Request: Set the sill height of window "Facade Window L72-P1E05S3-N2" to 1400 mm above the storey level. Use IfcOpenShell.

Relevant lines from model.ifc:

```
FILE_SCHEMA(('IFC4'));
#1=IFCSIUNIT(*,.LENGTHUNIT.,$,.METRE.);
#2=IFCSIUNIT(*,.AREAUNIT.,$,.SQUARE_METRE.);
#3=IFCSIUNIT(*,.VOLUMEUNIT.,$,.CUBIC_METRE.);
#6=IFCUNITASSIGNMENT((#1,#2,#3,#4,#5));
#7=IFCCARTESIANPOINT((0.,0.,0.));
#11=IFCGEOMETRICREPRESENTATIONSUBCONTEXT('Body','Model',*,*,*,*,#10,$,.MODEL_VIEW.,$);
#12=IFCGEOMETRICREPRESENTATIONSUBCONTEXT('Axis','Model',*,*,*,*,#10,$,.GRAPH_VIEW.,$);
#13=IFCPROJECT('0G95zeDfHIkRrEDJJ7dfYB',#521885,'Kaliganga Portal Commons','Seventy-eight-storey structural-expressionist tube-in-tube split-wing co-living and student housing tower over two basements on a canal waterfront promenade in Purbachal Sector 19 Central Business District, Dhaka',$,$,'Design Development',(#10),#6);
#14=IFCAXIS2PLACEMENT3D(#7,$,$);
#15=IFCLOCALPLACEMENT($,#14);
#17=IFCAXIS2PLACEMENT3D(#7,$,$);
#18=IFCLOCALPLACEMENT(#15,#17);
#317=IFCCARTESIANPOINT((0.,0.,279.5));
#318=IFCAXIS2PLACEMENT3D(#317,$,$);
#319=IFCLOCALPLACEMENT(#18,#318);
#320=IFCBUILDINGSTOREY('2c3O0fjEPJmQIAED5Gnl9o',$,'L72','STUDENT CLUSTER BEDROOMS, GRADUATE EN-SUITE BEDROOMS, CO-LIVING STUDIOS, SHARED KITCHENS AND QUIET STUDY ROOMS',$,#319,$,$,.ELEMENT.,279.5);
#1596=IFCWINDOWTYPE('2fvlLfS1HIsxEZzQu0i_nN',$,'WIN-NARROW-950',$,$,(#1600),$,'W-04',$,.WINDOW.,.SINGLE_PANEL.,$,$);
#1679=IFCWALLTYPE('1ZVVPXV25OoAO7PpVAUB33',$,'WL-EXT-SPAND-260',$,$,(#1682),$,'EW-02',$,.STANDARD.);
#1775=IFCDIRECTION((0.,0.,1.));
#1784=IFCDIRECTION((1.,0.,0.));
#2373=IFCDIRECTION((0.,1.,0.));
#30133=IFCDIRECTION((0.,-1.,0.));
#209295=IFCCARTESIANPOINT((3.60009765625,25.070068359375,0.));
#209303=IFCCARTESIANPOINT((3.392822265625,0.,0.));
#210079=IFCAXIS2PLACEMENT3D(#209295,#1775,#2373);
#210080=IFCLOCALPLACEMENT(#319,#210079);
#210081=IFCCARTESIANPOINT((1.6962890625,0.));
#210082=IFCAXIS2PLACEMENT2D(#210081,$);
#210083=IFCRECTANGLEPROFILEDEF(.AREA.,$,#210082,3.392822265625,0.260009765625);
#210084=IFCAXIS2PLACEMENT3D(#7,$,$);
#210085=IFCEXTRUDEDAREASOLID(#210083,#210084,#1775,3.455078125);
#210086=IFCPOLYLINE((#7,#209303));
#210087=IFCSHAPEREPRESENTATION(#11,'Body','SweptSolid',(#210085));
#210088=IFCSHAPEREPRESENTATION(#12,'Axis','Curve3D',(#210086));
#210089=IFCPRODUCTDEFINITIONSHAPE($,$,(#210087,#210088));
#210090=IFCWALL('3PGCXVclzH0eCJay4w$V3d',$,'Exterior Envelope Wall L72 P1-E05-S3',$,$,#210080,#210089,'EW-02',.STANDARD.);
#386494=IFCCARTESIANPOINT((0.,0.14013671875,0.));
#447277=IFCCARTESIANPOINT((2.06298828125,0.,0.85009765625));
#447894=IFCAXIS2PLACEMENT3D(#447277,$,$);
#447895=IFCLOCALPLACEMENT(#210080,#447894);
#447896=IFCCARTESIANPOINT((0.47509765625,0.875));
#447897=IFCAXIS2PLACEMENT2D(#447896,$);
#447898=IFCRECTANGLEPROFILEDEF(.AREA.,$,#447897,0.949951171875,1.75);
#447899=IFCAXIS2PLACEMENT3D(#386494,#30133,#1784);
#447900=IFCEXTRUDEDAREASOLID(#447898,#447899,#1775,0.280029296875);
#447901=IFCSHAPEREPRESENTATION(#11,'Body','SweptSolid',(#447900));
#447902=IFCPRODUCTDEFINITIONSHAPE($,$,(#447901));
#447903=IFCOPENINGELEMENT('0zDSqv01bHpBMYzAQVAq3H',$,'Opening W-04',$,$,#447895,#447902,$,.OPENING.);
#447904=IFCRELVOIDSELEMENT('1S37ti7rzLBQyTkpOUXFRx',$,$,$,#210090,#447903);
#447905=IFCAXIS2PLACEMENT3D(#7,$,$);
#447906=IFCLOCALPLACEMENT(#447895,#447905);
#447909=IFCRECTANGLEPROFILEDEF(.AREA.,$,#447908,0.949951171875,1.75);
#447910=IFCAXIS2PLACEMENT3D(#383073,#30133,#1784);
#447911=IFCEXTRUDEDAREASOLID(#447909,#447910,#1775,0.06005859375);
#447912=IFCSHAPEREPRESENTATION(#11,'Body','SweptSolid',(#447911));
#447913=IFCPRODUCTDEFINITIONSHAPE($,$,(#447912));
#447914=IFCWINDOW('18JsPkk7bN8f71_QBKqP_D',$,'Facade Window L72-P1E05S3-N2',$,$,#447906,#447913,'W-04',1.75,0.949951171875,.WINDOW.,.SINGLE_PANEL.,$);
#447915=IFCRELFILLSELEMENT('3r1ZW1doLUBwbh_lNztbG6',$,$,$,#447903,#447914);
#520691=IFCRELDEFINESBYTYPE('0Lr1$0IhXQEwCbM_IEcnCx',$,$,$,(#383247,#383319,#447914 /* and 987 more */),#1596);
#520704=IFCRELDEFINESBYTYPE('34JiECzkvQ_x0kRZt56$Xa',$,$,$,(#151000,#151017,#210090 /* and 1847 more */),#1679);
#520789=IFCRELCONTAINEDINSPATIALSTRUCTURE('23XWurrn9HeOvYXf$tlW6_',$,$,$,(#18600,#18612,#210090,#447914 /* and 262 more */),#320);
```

```python
import numpy as np
import ifcopenshell
import ifcopenshell.api.geometry
import ifcopenshell.geom
import ifcopenshell.util.element
import ifcopenshell.util.placement
import ifcopenshell.util.shape
import ifcopenshell.util.unit

model = ifcopenshell.open("model.ifc")
unit_scale = ifcopenshell.util.unit.calculate_unit_scale(model)

window = model.by_guid("18JsPkk7bN8f71_QBKqP_D")
opening = window.FillsVoids[0].RelatingOpeningElement
storey = ifcopenshell.util.element.get_container(window, ifc_class="IfcBuildingStorey")
level = ifcopenshell.util.placement.get_local_placement(storey.ObjectPlacement)[2, 3]

# The opening's origin need not be at the sill, so measure its lowest point.
shape = ifcopenshell.geom.create_shape(ifcopenshell.geom.settings(), opening)
bottom = ifcopenshell.util.shape.get_shape_bottom_elevation(shape, shape.geometry) / unit_scale
dz = level + 1.4 - bottom

shift = np.array([0.0, 0.0, dz])
# The window is placed relative to its opening, so it follows when the opening moves.
matrix = ifcopenshell.util.placement.get_local_placement(opening.ObjectPlacement)
matrix[:3, 3] += shift
ifcopenshell.api.geometry.edit_object_placement(
    model, product=opening, matrix=matrix, is_si=False, should_transform_children=True
)

print(f"moved by {dz * unit_scale:+.3f} m")

model.write("model_v2.ifc")
```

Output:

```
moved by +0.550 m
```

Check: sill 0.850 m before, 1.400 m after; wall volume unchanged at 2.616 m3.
